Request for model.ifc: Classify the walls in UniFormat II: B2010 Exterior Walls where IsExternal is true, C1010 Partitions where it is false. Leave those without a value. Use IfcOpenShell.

First a look at what the model holds.

```python
import ifcopenshell
import ifcopenshell.util.element

model = ifcopenshell.open("model.ifc")
print(model.schema)
print("classifications:", [c.Name for c in model.by_type("IfcClassification")])
values = [ifcopenshell.util.element.get_pset(e, "Pset_WallCommon", "IsExternal") for e in model.by_type("IfcWall")]
for value in (True, False, None):
    print("IsExternal", value, values.count(value))
```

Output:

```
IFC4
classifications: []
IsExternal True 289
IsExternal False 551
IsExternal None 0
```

```python
import ifcopenshell
import ifcopenshell.api.classification
import ifcopenshell.util.element

model = ifcopenshell.open("model.ifc")

system = ifcopenshell.api.classification.add_classification(model, classification="UniFormat II")

walls = model.by_type("IfcWall")
external = {e: ifcopenshell.util.element.get_pset(e, "Pset_WallCommon", "IsExternal") for e in walls}
for flag, code, name in ((True, "B2010", "Exterior Walls"), (False, "C1010", "Partitions")):
    products = [e for e in walls if external[e] is flag]
    ifcopenshell.api.classification.add_reference(
        model, products=products, classification=system, identification=code, name=name
    )
    print(code, len(products))

model.write("model_v2.ifc")
```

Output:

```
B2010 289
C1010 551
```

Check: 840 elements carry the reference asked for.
